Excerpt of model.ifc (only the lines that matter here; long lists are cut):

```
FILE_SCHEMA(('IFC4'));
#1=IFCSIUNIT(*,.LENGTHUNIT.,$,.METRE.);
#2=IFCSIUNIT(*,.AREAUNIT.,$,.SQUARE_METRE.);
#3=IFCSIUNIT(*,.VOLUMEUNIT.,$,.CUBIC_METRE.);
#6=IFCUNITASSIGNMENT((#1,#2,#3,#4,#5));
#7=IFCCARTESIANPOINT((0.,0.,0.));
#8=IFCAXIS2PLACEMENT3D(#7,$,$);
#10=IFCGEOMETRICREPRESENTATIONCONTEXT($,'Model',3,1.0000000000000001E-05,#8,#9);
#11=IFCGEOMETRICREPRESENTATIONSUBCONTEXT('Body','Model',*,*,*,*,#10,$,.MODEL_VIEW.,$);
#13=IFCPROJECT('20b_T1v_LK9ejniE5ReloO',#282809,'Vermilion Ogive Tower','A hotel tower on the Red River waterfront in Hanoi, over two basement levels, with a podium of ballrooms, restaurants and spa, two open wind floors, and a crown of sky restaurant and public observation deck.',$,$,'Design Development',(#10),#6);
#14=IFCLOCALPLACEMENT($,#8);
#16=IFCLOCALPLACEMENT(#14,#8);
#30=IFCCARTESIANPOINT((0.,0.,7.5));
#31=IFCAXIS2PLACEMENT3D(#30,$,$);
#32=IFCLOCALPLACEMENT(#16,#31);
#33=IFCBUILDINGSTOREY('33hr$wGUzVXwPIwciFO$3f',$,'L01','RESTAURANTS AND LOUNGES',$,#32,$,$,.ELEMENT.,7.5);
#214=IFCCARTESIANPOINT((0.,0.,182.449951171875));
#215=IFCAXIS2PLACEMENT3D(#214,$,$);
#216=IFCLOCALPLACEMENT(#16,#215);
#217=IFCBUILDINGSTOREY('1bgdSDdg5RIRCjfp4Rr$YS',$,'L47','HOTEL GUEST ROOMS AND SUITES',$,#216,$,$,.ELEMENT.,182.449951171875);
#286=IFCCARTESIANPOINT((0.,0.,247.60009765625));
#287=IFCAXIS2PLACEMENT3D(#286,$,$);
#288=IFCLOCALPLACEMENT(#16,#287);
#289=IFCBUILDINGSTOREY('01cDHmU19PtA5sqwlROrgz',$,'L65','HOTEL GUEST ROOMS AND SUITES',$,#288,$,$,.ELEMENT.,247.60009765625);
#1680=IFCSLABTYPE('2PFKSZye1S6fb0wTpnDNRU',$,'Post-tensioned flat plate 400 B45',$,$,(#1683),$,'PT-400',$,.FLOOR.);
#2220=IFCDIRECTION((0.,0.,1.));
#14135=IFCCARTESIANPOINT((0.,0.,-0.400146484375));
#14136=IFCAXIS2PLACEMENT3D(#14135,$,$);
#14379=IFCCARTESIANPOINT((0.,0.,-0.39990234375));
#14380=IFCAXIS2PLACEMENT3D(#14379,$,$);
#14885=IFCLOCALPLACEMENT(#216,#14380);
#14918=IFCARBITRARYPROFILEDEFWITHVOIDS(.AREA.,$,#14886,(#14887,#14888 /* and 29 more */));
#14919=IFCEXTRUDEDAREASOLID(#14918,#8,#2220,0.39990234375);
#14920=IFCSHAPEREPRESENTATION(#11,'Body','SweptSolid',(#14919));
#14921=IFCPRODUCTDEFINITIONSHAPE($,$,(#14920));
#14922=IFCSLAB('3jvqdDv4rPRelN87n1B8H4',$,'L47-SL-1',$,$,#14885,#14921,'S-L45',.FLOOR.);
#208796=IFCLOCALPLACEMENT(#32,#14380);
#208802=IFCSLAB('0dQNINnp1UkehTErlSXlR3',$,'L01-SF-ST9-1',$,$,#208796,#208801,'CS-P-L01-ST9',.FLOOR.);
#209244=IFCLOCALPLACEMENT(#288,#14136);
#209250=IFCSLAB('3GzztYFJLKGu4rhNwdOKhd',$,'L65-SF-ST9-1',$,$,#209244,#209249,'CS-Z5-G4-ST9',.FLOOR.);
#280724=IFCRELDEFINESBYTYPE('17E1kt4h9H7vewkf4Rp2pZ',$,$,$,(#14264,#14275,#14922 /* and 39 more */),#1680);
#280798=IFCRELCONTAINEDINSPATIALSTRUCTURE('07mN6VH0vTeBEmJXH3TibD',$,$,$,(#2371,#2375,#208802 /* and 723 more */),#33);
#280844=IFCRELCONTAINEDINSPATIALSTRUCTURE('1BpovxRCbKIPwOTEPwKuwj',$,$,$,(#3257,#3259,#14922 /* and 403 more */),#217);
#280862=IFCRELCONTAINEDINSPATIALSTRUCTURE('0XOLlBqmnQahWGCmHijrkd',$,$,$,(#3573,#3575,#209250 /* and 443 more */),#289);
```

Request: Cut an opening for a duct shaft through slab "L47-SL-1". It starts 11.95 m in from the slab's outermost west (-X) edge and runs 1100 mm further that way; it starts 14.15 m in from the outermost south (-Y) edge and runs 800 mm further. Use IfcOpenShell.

```python
import numpy as np
import ifcopenshell
import ifcopenshell.api.feature
import ifcopenshell.api.geometry
import ifcopenshell.api.root
import ifcopenshell.geom
import ifcopenshell.util.placement
import ifcopenshell.util.representation
import ifcopenshell.util.shape
import ifcopenshell.util.unit

model = ifcopenshell.open("model.ifc")
unit_scale = ifcopenshell.util.unit.calculate_unit_scale(model)
settings = ifcopenshell.geom.settings()


def volume(element):
    """Net volume in cubic metres, openings subtracted."""
    shape = ifcopenshell.geom.create_shape(settings, element)
    return ifcopenshell.util.shape.get_volume(shape.geometry)


slab = model.by_guid("3jvqdDv4rPRelN87n1B8H4")
before = volume(slab)

# Extent in the slab's own axes, in metres. The edges named are its -X and -Y sides.
slab_shape = ifcopenshell.geom.create_shape(settings, slab)
vertices = ifcopenshell.util.shape.get_vertices(slab_shape.geometry)
x_min, y_min, bottom = vertices.min(axis=0)
top = vertices[:, 2].max()

opening = ifcopenshell.api.root.create_entity(model, ifc_class="IfcOpeningElement", name="Duct shaft opening", predefined_type="OPENING")
context = ifcopenshell.util.representation.get_context(model, "Model", "Body", "MODEL_VIEW")
width, depth = 1.1, 0.8
outline = [(0.0, 0.0), (width, 0.0), (width, depth), (0.0, depth), (0.0, 0.0)]
# Overshoot both faces by 50 mm so the cut is clean.
shape = ifcopenshell.api.geometry.add_slab_representation(
    model, context=context, depth=top - bottom + 0.1, polyline=outline
)
ifcopenshell.api.geometry.assign_representation(model, product=opening, representation=shape)

matrix = ifcopenshell.util.placement.get_local_placement(slab.ObjectPlacement)
matrix[:, 3] = matrix @ np.append(np.array([x_min + 11.95, y_min + 14.15, bottom - 0.05]) / unit_scale, 1.0)
ifcopenshell.api.geometry.edit_object_placement(model, product=opening, matrix=matrix, is_si=False)
ifcopenshell.api.feature.add_feature(model, feature=opening, element=slab)

after = volume(slab)

print(f"slab volume {before:.3f} -> {after:.3f} m3")

model.write("model_updated.ifc")
```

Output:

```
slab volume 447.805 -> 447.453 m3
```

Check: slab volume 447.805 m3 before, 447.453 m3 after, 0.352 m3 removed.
